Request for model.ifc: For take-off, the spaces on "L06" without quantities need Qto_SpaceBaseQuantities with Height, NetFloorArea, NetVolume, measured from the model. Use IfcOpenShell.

First a look at what the model holds.

```python
import ifcopenshell
import ifcopenshell.util.element
import ifcopenshell.util.unit

model = ifcopenshell.open("model.ifc")
print(model.schema)
for unit_type in ("LENGTHUNIT", "AREAUNIT", "VOLUMEUNIT"):
    print(unit_type, ifcopenshell.util.unit.calculate_unit_scale(model, unit_type))
storey = next(s for s in model.by_type("IfcBuildingStorey") if s.Name == "L06")
spaces = [e for e in ifcopenshell.util.element.get_decomposition(storey) if e.is_a("IfcSpace")]
for e in sorted(spaces, key=lambda e: e.id()):
    print(e.id(), e.is_a(), e.Name, list(ifcopenshell.util.element.get_psets(e, qtos_only=True)), sep=" | ")
```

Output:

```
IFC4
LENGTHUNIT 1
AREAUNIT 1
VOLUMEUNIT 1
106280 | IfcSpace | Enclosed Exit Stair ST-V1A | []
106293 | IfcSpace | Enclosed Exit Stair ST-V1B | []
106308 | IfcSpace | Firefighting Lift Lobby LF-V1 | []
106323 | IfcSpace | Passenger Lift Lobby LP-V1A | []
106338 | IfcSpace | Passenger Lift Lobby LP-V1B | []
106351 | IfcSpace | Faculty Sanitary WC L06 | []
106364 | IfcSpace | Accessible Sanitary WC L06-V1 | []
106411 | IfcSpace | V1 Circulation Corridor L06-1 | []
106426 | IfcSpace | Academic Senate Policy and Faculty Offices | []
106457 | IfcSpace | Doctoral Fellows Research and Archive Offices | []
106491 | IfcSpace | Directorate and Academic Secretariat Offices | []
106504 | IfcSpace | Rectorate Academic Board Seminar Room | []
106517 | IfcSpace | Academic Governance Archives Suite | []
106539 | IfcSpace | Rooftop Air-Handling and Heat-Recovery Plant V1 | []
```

```python
import ifcopenshell
import ifcopenshell.api.pset
import ifcopenshell.geom
import ifcopenshell.util.element
import ifcopenshell.util.shape
import ifcopenshell.util.unit

model = ifcopenshell.open("model.ifc")
unit_scale = ifcopenshell.util.unit.calculate_unit_scale(model)
area_scale = ifcopenshell.util.unit.calculate_unit_scale(model, "AREAUNIT")
volume_scale = ifcopenshell.util.unit.calculate_unit_scale(model, "VOLUMEUNIT")
settings = ifcopenshell.geom.settings()

storey = next(s for s in model.by_type("IfcBuildingStorey") if s.Name == "L06")
spaces = [e for e in ifcopenshell.util.element.get_decomposition(storey) if e.is_a("IfcSpace")]

for e in sorted(spaces, key=lambda e: e.id()):
    if ifcopenshell.util.element.get_psets(e, qtos_only=True, should_inherit=False):
        continue
    # Geometry comes back in metres, in the element's own axes.
    shape = ifcopenshell.geom.create_shape(settings, e)
    values = {
        "Height": ifcopenshell.util.shape.get_z(shape.geometry) / unit_scale,
        "NetFloorArea": ifcopenshell.util.shape.get_footprint_area(shape.geometry) / area_scale,
        "NetVolume": ifcopenshell.util.shape.get_volume(shape.geometry) / volume_scale,
    }
    qto = ifcopenshell.api.pset.add_qto(model, product=e, name="Qto_SpaceBaseQuantities")
    ifcopenshell.api.pset.edit_qto(model, qto=qto, properties=values)
    print(e.id(), {k: round(v, 3) for k, v in values.items()})

model.write("model_updated.ifc")
```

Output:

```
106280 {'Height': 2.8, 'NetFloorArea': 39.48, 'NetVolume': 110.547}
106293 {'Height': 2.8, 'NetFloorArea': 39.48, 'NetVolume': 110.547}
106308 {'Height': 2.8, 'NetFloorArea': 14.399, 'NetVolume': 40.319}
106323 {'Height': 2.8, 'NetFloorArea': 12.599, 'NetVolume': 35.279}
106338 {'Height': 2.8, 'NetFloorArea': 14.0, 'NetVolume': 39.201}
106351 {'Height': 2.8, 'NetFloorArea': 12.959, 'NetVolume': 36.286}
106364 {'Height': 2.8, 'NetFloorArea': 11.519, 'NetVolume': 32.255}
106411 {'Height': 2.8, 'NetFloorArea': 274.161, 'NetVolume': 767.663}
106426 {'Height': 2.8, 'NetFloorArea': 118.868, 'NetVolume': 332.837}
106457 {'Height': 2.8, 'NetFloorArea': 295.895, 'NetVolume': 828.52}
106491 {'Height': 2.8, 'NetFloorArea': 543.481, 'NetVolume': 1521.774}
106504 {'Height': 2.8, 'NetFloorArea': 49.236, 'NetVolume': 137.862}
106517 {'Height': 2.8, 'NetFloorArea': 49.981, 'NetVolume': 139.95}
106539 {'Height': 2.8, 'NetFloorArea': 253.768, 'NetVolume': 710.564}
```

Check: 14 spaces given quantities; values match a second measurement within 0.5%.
